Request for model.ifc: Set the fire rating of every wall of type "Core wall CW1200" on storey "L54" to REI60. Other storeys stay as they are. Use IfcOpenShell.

First a look at what the model holds.

```python
import ifcopenshell
import ifcopenshell.util.element

model = ifcopenshell.open("model.ifc")
print(model.schema)
storey = next(s for s in model.by_type("IfcBuildingStorey") if s.Name == "L54")
walls = [e for e in ifcopenshell.util.element.get_decomposition(storey) if e.is_a("IfcWall")]
seen = {}
for e in walls:
    element_type = ifcopenshell.util.element.get_type(e)
    key = (element_type.Name if element_type != e and element_type else None, ifcopenshell.util.element.get_pset(e, "Pset_WallCommon", "FireRating"))
    seen[key] = seen.get(key, 0) + 1
for (name, value), count in sorted(seen.items(), key=str):
    print(count, "x", name, "|", value)
```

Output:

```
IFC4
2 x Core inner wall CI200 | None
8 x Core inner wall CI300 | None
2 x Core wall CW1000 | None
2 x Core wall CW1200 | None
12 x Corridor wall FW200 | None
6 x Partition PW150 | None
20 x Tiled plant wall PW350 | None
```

```python
import ifcopenshell
import ifcopenshell.api.pset
import ifcopenshell.util.element

model = ifcopenshell.open("model.ifc")

storey = next(s for s in model.by_type("IfcBuildingStorey") if s.Name == "L54")
walls = [e for e in ifcopenshell.util.element.get_decomposition(storey) if e.is_a("IfcWall")]

count = 0
for e in walls:
    element_type = ifcopenshell.util.element.get_type(e)
    if element_type in (None, e) or element_type.Name != "Core wall CW1200":
        continue
    found = ifcopenshell.util.element.get_pset(e, "Pset_WallCommon", should_inherit=False)
    if found:
        pset = model.by_id(found["id"])
        if len(ifcopenshell.util.element.get_elements_by_pset(pset)) > 1:
            pset = ifcopenshell.api.pset.unshare_pset(model, products=[e], pset=pset)[0]
    else:
        pset = ifcopenshell.api.pset.add_pset(model, product=e, name="Pset_WallCommon")
    ifcopenshell.api.pset.edit_pset(model, pset=pset, properties={"FireRating": "REI60"})
    count += 1

print(count, "walls updated")

model.write("model_rev.ifc")
```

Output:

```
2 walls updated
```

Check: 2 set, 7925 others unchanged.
